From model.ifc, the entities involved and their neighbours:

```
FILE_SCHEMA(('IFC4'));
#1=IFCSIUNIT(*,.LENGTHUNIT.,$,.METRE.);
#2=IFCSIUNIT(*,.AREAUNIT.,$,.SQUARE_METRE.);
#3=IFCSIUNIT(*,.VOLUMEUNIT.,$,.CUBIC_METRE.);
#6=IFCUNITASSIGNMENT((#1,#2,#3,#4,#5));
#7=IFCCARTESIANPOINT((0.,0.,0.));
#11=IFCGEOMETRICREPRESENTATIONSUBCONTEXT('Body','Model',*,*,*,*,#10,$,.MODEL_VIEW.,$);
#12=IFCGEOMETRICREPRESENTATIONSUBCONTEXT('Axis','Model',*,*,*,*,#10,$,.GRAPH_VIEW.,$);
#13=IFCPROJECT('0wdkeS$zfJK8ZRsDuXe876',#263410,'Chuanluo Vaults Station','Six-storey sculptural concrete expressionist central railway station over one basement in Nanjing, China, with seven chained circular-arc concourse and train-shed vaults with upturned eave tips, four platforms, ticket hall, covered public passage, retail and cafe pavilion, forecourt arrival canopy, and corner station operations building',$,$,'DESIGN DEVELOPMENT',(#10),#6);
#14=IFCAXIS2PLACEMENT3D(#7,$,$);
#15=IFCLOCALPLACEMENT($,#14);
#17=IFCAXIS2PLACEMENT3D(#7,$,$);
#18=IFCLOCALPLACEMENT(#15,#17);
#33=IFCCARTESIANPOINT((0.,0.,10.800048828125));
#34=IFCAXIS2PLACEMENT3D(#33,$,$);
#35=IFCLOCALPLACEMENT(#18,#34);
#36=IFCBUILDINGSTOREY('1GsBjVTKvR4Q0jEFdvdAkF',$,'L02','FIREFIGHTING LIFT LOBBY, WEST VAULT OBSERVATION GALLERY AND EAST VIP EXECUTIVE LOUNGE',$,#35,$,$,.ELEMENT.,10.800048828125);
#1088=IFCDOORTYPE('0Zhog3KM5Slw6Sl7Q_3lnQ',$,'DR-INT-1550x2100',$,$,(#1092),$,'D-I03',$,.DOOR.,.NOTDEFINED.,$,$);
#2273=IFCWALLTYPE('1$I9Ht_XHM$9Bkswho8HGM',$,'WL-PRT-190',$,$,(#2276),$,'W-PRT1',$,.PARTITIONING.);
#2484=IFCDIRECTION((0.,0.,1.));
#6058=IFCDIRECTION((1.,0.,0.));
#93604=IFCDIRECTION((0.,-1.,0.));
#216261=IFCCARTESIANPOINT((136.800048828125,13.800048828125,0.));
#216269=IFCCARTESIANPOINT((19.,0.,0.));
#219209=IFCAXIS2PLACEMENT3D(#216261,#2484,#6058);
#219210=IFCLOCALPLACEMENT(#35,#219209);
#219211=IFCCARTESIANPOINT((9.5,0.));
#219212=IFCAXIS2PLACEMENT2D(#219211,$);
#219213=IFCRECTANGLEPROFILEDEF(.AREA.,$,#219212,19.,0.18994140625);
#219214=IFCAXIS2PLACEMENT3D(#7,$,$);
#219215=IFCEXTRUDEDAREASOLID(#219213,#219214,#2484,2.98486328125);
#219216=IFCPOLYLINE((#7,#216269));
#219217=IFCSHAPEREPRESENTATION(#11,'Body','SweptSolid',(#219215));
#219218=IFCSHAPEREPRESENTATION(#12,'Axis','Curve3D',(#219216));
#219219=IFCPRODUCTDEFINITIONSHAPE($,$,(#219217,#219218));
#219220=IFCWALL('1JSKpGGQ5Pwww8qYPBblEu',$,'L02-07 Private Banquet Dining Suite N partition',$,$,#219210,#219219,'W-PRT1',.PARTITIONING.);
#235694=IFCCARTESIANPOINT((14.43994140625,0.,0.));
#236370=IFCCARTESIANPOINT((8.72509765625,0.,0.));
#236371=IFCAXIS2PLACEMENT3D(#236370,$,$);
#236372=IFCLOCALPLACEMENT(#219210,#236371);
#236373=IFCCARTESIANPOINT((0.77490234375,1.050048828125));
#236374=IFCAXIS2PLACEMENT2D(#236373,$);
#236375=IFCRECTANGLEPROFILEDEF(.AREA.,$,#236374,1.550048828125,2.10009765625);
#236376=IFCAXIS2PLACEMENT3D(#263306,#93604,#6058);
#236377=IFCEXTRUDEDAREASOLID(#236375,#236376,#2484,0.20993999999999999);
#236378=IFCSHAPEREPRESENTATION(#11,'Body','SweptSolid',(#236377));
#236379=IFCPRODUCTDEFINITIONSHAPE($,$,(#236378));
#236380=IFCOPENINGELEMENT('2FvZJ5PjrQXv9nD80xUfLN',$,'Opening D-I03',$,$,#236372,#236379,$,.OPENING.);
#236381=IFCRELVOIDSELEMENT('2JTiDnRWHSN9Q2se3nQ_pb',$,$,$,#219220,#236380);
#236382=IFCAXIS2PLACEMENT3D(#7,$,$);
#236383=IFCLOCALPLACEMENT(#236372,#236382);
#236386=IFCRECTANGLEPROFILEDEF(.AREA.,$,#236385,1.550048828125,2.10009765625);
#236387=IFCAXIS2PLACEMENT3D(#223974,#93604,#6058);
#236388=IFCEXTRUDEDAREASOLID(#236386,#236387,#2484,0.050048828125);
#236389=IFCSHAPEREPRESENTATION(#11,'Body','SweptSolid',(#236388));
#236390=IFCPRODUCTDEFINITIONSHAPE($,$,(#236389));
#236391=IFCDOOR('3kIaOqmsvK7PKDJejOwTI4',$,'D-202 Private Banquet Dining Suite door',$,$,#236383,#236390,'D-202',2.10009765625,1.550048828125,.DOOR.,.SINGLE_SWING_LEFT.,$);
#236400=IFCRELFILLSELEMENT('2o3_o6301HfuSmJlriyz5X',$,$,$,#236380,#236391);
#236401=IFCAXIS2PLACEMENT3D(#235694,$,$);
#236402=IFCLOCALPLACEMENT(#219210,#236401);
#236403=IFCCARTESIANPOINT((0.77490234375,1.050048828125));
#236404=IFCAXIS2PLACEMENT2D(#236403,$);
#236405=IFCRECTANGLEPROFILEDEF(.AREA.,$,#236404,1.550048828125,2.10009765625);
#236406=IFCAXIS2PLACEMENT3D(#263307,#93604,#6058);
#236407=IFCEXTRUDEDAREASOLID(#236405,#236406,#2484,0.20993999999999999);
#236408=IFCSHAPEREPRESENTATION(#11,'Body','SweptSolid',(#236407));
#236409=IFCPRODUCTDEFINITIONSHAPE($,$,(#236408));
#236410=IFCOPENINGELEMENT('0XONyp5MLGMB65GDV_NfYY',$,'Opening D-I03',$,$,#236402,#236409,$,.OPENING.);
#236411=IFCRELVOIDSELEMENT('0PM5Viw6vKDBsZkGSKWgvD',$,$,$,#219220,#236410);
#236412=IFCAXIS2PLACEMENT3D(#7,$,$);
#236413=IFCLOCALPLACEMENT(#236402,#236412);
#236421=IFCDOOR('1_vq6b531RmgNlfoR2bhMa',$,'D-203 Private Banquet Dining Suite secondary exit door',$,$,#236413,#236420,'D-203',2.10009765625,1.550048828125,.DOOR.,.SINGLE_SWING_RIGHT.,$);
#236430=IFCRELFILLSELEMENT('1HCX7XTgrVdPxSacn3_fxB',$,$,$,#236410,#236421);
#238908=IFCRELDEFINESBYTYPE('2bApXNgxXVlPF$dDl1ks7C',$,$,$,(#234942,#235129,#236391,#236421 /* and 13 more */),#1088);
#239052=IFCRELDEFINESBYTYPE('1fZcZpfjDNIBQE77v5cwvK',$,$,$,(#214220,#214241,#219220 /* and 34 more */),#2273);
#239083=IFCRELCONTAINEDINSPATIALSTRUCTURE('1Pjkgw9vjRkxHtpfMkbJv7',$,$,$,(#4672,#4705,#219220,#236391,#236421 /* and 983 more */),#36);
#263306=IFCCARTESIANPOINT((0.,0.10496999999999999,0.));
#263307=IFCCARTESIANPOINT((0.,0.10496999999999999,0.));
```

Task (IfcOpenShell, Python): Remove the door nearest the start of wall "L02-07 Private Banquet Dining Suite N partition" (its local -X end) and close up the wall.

```python
import ifcopenshell
import ifcopenshell.api.feature
import ifcopenshell.api.root
import ifcopenshell.geom
import ifcopenshell.util.shape

model = ifcopenshell.open("model.ifc")
settings = ifcopenshell.geom.settings()


def volume(element):
    """Net volume in cubic metres, openings subtracted."""
    shape = ifcopenshell.geom.create_shape(settings, element)
    return ifcopenshell.util.shape.get_volume(shape.geometry)


door = model.by_guid("3kIaOqmsvK7PKDJejOwTI4")
opening = door.FillsVoids[0].RelatingOpeningElement
wall = opening.VoidsElements[0].RelatingBuildingElement
before = volume(wall)

ifcopenshell.api.root.remove_product(model, product=door)
ifcopenshell.api.feature.remove_feature(model, feature=opening)

after = volume(wall)

print(f"wall volume {before:.3f} -> {after:.3f} m3")

model.write("model-out.ifc")
```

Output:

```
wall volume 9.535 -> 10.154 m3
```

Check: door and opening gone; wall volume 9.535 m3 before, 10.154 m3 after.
